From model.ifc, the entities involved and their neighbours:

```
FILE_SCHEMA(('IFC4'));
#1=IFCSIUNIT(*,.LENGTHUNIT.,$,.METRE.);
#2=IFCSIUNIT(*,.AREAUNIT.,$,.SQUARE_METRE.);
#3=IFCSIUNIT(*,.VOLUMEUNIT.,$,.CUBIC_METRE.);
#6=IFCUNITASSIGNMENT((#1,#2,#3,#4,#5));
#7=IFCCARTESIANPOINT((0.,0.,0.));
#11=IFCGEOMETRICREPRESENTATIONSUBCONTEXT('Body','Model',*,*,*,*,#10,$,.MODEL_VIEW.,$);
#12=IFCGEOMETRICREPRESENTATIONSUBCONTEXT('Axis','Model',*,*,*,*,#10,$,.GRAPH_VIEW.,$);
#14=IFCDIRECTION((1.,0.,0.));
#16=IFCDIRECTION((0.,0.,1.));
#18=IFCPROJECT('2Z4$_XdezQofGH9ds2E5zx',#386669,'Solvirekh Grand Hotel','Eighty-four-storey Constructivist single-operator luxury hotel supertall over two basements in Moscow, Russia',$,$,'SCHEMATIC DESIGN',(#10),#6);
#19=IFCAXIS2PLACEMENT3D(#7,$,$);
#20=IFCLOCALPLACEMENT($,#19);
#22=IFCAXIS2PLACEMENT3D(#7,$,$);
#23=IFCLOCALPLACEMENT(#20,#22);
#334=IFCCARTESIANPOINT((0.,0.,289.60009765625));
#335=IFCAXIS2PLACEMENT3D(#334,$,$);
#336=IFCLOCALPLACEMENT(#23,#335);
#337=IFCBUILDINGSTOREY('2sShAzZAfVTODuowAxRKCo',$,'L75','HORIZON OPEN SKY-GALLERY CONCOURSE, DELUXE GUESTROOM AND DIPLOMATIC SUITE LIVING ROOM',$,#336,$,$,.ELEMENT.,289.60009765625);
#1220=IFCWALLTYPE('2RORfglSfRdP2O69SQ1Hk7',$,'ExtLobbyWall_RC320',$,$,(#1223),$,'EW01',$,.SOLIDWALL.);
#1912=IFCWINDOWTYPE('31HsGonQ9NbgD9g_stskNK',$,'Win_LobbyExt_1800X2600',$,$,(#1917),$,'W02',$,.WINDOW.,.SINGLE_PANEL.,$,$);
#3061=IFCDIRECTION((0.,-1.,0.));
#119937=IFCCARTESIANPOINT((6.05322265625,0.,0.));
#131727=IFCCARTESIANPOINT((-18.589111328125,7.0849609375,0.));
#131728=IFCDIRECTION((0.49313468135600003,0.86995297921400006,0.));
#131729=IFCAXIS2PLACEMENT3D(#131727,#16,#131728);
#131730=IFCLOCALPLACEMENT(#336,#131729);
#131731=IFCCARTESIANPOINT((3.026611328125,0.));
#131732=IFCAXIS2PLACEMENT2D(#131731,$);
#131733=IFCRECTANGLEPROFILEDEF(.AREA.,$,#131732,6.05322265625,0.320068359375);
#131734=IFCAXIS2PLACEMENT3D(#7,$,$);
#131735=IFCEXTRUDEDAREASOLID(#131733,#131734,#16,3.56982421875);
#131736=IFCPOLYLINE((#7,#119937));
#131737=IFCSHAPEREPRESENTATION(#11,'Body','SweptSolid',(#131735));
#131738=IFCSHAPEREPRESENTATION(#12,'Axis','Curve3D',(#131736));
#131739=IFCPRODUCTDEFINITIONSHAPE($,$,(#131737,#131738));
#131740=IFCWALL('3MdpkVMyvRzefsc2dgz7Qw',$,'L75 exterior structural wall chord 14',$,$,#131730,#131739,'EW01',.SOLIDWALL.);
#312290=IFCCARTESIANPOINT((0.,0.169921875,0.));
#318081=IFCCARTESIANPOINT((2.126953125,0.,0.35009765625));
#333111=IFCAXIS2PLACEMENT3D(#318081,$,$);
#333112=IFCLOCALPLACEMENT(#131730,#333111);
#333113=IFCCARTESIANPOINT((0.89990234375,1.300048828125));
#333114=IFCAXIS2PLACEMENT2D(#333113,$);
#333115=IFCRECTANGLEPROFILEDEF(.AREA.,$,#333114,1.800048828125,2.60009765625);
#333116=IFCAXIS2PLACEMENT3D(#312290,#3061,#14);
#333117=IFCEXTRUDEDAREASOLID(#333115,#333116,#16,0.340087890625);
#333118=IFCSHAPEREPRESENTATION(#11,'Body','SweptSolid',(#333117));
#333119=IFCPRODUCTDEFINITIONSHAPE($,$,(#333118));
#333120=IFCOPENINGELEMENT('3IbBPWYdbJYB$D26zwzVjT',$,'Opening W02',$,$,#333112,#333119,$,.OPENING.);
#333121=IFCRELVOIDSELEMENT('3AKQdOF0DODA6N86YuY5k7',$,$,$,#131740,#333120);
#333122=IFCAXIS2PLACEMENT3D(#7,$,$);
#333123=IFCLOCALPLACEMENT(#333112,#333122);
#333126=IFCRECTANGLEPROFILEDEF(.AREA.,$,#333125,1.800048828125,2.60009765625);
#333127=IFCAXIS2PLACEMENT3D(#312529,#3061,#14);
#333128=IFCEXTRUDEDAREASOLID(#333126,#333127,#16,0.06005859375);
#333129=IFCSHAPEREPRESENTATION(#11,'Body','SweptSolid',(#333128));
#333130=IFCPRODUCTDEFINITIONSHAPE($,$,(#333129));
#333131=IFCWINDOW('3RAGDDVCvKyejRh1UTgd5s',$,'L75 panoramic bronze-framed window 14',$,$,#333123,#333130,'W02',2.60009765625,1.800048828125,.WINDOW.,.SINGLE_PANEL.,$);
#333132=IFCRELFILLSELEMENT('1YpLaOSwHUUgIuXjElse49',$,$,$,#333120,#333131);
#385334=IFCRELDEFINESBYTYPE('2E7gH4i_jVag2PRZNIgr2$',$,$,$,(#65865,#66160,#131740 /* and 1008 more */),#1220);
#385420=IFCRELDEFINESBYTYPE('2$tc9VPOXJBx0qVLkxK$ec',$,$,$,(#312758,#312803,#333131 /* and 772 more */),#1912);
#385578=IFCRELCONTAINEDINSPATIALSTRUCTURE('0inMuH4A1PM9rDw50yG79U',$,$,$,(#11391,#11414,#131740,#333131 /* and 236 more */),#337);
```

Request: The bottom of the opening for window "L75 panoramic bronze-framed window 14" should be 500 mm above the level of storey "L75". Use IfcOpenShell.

```python
import numpy as np
import ifcopenshell
import ifcopenshell.api.geometry
import ifcopenshell.geom
import ifcopenshell.util.element
import ifcopenshell.util.placement
import ifcopenshell.util.shape
import ifcopenshell.util.unit

model = ifcopenshell.open("model.ifc")
unit_scale = ifcopenshell.util.unit.calculate_unit_scale(model)

window = model.by_guid("3RAGDDVCvKyejRh1UTgd5s")
opening = window.FillsVoids[0].RelatingOpeningElement
storey = ifcopenshell.util.element.get_container(window, ifc_class="IfcBuildingStorey")
level = ifcopenshell.util.placement.get_local_placement(storey.ObjectPlacement)[2, 3]

# The opening's origin need not be at the sill, so measure its lowest point.
shape = ifcopenshell.geom.create_shape(ifcopenshell.geom.settings(), opening)
bottom = ifcopenshell.util.shape.get_shape_bottom_elevation(shape, shape.geometry) / unit_scale
dz = level + 0.5 - bottom

shift = np.array([0.0, 0.0, dz])
# The window is placed relative to its opening, so it follows when the opening moves.
matrix = ifcopenshell.util.placement.get_local_placement(opening.ObjectPlacement)
matrix[:3, 3] += shift
ifcopenshell.api.geometry.edit_object_placement(
    model, product=opening, matrix=matrix, is_si=False, should_transform_children=True
)

print(f"moved by {dz * unit_scale:+.3f} m")

model.write("model-out.ifc")
```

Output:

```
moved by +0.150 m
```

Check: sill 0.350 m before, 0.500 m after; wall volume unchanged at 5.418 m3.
